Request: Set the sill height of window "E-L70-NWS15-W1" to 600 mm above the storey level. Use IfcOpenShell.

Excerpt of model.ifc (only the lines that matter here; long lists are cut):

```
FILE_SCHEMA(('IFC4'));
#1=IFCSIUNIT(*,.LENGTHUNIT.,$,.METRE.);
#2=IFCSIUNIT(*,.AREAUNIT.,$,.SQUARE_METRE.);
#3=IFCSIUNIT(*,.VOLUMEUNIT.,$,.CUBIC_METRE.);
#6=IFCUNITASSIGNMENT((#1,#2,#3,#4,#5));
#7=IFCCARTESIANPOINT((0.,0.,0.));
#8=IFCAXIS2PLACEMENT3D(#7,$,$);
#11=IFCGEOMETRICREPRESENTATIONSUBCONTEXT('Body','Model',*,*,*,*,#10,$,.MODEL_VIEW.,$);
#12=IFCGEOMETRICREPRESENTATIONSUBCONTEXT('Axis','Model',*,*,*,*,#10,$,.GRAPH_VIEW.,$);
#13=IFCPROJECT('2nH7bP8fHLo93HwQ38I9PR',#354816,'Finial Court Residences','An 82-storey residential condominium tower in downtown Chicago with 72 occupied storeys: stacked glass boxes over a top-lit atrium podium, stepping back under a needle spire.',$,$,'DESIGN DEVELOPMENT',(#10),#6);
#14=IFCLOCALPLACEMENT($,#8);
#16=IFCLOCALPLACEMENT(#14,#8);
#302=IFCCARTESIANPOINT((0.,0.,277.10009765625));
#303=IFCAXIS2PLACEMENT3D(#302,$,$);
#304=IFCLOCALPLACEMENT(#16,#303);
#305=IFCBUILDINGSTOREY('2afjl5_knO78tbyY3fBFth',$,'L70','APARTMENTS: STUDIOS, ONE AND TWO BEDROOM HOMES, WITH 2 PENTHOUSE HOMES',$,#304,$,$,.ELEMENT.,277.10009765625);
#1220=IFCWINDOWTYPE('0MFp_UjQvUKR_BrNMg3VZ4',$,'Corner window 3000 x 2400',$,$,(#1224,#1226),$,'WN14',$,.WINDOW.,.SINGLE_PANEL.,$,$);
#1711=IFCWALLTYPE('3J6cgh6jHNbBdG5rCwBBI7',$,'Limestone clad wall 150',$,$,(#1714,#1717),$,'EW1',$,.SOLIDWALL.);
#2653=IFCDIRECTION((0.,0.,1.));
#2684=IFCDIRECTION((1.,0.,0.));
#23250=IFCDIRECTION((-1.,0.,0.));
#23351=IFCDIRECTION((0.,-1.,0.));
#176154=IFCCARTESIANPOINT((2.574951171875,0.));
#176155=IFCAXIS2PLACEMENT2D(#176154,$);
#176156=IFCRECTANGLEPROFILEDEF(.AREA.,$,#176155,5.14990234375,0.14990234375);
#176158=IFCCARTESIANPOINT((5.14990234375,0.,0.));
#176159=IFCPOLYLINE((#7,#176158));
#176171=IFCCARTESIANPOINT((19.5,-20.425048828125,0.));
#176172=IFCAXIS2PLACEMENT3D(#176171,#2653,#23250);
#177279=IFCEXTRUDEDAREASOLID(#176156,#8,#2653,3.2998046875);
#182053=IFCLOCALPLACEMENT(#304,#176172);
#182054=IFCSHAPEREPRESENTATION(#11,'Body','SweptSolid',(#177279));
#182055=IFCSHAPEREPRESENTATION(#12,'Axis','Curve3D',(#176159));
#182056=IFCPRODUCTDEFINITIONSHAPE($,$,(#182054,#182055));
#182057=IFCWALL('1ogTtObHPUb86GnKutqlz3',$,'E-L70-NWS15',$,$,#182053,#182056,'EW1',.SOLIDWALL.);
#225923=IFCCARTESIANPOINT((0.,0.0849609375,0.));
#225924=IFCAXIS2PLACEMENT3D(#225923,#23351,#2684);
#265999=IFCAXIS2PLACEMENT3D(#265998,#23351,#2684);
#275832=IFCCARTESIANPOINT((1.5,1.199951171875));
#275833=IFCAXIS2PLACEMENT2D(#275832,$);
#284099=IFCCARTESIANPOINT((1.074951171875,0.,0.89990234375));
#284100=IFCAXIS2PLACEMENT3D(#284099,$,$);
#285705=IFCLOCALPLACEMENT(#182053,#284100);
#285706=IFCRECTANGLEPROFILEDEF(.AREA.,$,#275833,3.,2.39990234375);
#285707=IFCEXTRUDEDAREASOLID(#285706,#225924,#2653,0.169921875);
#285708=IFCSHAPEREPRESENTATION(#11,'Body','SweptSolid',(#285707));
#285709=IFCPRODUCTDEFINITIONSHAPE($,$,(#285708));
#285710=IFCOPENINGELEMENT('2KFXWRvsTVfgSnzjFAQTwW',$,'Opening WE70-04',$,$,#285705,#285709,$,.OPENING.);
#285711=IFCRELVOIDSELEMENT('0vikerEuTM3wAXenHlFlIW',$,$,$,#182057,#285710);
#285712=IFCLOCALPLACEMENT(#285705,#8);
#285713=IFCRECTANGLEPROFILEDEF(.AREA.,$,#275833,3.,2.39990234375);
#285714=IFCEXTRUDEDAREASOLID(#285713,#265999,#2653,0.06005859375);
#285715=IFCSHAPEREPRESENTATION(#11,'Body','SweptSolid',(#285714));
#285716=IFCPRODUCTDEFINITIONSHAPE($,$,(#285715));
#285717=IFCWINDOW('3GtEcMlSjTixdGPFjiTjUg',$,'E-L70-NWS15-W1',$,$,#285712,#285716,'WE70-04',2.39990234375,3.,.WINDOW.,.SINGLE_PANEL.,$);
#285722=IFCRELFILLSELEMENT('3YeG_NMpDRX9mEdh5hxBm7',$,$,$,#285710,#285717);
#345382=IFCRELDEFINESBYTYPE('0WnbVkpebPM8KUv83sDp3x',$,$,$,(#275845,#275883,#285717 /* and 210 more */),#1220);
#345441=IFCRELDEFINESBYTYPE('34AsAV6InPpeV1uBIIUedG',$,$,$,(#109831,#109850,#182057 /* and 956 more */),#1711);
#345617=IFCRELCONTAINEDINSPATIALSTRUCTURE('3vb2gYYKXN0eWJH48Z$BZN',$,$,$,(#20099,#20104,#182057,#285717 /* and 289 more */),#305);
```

```python
import numpy as np
import ifcopenshell
import ifcopenshell.api.geometry
import ifcopenshell.geom
import ifcopenshell.util.element
import ifcopenshell.util.placement
import ifcopenshell.util.shape
import ifcopenshell.util.unit

model = ifcopenshell.open("model.ifc")
unit_scale = ifcopenshell.util.unit.calculate_unit_scale(model)

window = model.by_guid("3GtEcMlSjTixdGPFjiTjUg")
opening = window.FillsVoids[0].RelatingOpeningElement
storey = ifcopenshell.util.element.get_container(window, ifc_class="IfcBuildingStorey")
level = ifcopenshell.util.placement.get_local_placement(storey.ObjectPlacement)[2, 3]

# The opening's origin need not be at the sill, so measure its lowest point.
shape = ifcopenshell.geom.create_shape(ifcopenshell.geom.settings(), opening)
bottom = ifcopenshell.util.shape.get_shape_bottom_elevation(shape, shape.geometry) / unit_scale
dz = level + 0.6 / unit_scale - bottom

shift = np.array([0.0, 0.0, dz])
# The window is placed relative to its opening, so it follows when the opening moves.
matrix = ifcopenshell.util.placement.get_local_placement(opening.ObjectPlacement)
matrix[:3, 3] += shift
ifcopenshell.api.geometry.edit_object_placement(
    model, product=opening, matrix=matrix, is_si=False, should_transform_children=True
)

print(f"moved by {dz * unit_scale:+.3f} m")

model.write("model_updated.ifc")
```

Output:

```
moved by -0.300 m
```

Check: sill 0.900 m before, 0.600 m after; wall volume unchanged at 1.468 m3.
